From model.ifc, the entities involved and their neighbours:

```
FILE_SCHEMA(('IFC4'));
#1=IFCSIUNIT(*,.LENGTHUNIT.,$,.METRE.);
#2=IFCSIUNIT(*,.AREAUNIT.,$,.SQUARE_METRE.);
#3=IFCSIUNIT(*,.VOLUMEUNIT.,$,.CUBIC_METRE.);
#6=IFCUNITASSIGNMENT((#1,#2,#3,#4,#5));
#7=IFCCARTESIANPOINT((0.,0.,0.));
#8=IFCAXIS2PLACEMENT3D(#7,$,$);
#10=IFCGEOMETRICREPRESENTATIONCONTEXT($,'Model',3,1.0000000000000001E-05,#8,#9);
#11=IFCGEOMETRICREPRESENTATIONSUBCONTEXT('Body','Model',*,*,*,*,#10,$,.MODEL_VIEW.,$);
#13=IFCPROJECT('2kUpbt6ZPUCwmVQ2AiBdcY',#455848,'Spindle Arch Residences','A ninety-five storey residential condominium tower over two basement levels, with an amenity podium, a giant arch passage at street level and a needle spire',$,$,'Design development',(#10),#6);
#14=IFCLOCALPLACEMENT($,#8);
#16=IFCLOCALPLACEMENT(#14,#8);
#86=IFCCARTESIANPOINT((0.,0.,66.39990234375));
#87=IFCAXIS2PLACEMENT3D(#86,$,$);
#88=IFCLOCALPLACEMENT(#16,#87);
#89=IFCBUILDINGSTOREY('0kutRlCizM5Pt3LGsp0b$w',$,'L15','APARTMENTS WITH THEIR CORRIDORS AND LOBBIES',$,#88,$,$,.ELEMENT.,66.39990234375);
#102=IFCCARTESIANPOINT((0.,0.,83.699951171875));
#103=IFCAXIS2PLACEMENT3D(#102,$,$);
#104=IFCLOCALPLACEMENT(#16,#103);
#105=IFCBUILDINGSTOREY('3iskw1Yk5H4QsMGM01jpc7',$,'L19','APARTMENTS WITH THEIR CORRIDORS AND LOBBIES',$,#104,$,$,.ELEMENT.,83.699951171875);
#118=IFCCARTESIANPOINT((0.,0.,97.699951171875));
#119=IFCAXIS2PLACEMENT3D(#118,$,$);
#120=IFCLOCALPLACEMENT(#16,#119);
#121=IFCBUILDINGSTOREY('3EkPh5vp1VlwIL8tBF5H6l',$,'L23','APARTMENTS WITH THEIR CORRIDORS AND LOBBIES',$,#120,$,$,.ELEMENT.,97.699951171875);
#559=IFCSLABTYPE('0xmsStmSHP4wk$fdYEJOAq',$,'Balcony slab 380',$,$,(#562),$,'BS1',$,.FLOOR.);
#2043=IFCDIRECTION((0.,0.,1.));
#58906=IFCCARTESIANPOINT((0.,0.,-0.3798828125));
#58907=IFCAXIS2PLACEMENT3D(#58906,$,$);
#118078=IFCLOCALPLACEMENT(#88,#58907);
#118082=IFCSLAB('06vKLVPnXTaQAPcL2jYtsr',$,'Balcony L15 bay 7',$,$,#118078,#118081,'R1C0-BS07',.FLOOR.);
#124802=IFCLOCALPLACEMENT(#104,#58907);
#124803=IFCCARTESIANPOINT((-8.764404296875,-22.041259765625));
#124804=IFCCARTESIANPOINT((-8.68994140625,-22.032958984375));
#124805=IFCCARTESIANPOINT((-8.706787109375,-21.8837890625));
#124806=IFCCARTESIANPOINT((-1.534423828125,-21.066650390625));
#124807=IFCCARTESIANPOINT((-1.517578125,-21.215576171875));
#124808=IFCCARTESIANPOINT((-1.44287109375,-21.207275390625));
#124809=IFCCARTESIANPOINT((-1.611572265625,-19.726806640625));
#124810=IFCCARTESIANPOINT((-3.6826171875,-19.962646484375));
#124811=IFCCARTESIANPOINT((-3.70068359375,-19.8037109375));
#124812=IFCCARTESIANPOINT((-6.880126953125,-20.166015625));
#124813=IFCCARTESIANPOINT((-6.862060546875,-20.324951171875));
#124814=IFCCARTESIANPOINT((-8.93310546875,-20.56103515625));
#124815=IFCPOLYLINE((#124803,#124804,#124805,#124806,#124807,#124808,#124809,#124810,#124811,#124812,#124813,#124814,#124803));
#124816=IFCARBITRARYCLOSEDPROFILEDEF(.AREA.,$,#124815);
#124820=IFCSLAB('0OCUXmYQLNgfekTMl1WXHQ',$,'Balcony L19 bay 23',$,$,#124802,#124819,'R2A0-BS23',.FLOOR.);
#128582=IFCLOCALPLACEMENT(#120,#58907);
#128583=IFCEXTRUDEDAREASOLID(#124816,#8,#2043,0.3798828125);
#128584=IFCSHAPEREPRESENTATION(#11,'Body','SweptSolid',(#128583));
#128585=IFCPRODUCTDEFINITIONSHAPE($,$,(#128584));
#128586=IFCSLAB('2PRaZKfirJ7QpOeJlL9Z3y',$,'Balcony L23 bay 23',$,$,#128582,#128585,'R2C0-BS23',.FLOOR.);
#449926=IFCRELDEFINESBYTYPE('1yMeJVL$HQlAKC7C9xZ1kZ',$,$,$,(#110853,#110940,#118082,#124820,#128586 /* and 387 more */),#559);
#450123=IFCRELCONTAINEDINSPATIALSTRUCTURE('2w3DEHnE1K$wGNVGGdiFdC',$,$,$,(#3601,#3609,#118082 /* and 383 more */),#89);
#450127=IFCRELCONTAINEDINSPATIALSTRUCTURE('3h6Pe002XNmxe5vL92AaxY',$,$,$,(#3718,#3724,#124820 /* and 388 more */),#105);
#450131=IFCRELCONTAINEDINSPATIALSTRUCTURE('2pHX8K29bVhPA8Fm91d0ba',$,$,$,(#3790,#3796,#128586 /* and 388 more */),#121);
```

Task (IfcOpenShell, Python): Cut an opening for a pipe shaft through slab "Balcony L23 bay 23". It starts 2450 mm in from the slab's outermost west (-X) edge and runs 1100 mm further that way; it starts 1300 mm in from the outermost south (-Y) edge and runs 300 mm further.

```python
import numpy as np
import ifcopenshell
import ifcopenshell.api.feature
import ifcopenshell.api.geometry
import ifcopenshell.api.root
import ifcopenshell.geom
import ifcopenshell.util.placement
import ifcopenshell.util.representation
import ifcopenshell.util.shape
import ifcopenshell.util.unit

model = ifcopenshell.open("model.ifc")
unit_scale = ifcopenshell.util.unit.calculate_unit_scale(model)
settings = ifcopenshell.geom.settings()


def volume(element):
    """Net volume in cubic metres, openings subtracted."""
    shape = ifcopenshell.geom.create_shape(settings, element)
    return ifcopenshell.util.shape.get_volume(shape.geometry)


slab = model.by_id(128586)
before = volume(slab)

# Extent in the slab's own axes, in metres. The edges named are its -X and -Y sides.
slab_shape = ifcopenshell.geom.create_shape(settings, slab)
vertices = ifcopenshell.util.shape.get_vertices(slab_shape.geometry)
x_min, y_min, bottom = vertices.min(axis=0)
top = vertices[:, 2].max()

opening = ifcopenshell.api.root.create_entity(model, ifc_class="IfcOpeningElement", name="Pipe shaft opening", predefined_type="OPENING")
context = ifcopenshell.util.representation.get_context(model, "Model", "Body", "MODEL_VIEW")
width, depth = 1.1, 0.3
outline = [(0.0, 0.0), (width, 0.0), (width, depth), (0.0, depth), (0.0, 0.0)]
# Overshoot both faces by 50 mm so the cut is clean.
shape = ifcopenshell.api.geometry.add_slab_representation(
    model, context=context, depth=top - bottom + 0.1, polyline=outline
)
ifcopenshell.api.geometry.assign_representation(model, product=opening, representation=shape)

matrix = ifcopenshell.util.placement.get_local_placement(slab.ObjectPlacement)
matrix[:, 3] = matrix @ np.append(np.array([x_min + 2.45, y_min + 1.3, bottom - 0.05]) / unit_scale, 1.0)
ifcopenshell.api.geometry.edit_object_placement(model, product=opening, matrix=matrix, is_si=False)
ifcopenshell.api.feature.add_feature(model, feature=opening, element=slab)

after = volume(slab)

print(f"slab volume {before:.3f} -> {after:.3f} m3")

model.write("model-out.ifc")
```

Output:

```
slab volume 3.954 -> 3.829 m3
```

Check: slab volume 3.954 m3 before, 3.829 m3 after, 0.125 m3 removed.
